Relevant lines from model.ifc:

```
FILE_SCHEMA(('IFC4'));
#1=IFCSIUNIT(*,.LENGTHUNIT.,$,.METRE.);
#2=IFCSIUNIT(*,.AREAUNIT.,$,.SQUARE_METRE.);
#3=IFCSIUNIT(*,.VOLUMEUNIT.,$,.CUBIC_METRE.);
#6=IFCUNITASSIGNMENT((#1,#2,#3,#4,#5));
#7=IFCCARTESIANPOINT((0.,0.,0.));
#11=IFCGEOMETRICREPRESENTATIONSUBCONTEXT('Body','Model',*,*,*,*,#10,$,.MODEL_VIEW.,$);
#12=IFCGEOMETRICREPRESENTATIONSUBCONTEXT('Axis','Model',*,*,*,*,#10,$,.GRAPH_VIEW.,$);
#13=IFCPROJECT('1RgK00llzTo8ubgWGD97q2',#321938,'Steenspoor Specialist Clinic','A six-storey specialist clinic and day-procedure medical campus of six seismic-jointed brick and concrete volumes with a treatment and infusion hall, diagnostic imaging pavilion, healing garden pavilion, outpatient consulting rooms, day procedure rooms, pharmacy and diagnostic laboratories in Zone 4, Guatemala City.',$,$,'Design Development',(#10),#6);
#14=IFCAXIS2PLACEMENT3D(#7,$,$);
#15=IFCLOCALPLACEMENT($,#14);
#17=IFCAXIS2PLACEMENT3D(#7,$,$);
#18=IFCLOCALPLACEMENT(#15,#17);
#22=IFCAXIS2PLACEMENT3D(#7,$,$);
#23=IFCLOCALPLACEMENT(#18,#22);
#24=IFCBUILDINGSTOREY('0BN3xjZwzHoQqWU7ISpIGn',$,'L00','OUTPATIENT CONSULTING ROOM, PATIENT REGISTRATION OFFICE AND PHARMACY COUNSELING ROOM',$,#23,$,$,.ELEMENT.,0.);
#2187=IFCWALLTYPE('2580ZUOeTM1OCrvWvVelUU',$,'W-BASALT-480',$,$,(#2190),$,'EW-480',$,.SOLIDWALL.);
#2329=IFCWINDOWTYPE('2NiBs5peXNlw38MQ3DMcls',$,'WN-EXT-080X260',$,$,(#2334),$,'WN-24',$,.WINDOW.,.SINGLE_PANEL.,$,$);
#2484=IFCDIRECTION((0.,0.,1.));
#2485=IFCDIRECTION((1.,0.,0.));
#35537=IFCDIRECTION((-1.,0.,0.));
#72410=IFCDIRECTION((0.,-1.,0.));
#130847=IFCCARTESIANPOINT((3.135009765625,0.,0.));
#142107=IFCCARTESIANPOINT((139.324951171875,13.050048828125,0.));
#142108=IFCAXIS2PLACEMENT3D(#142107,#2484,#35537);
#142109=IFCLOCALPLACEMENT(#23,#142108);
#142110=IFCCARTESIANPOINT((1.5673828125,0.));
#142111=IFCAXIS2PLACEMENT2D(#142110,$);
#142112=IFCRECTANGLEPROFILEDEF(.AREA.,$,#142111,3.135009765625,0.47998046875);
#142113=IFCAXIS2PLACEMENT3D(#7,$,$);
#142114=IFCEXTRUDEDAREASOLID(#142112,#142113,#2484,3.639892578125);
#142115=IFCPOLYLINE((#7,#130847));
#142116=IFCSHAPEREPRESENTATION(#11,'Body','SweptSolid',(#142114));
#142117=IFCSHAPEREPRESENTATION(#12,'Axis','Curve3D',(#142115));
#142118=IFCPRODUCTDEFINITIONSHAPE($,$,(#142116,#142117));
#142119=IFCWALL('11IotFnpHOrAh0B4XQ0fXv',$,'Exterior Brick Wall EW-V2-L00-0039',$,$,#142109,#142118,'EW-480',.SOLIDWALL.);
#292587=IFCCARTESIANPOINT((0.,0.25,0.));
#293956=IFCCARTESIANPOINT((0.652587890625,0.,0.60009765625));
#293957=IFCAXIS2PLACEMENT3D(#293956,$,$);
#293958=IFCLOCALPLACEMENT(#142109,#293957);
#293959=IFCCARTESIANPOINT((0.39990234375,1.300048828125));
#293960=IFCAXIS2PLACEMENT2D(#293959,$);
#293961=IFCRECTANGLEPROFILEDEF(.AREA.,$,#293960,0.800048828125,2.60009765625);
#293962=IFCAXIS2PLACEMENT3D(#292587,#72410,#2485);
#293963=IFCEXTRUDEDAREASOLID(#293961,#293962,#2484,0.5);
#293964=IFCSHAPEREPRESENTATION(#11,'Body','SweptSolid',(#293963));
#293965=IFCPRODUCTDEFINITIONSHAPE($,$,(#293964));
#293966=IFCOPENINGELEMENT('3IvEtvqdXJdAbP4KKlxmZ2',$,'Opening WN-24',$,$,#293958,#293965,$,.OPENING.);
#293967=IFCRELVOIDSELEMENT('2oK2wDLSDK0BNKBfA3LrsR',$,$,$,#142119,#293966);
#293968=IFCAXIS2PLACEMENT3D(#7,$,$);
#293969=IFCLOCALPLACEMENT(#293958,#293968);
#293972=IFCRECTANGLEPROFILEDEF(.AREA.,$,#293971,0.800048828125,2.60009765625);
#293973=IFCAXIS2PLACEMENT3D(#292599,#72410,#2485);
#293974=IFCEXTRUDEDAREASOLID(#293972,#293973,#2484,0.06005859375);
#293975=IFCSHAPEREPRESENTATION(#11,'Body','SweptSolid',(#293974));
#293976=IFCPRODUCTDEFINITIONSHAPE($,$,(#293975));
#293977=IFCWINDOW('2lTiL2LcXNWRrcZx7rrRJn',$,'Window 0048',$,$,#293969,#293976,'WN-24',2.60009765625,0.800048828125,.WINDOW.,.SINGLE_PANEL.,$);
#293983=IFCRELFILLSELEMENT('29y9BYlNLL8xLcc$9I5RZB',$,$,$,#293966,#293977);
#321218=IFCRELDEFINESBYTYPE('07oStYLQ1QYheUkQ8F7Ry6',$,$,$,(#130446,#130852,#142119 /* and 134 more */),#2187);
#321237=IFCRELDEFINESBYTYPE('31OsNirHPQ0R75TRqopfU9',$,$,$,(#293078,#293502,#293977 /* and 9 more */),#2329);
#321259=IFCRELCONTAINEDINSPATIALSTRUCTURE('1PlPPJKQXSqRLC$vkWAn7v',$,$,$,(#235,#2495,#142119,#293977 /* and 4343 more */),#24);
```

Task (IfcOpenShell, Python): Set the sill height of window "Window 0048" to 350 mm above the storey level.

```python
import numpy as np
import ifcopenshell
import ifcopenshell.api.geometry
import ifcopenshell.geom
import ifcopenshell.util.element
import ifcopenshell.util.placement
import ifcopenshell.util.shape
import ifcopenshell.util.unit

model = ifcopenshell.open("model.ifc")
unit_scale = ifcopenshell.util.unit.calculate_unit_scale(model)

window = model.by_guid("2lTiL2LcXNWRrcZx7rrRJn")
opening = window.FillsVoids[0].RelatingOpeningElement
storey = ifcopenshell.util.element.get_container(window, ifc_class="IfcBuildingStorey")
level = ifcopenshell.util.placement.get_local_placement(storey.ObjectPlacement)[2, 3]

# The opening's origin need not be at the sill, so measure its lowest point.
shape = ifcopenshell.geom.create_shape(ifcopenshell.geom.settings(), opening)
bottom = ifcopenshell.util.shape.get_shape_bottom_elevation(shape, shape.geometry) / unit_scale
dz = level + 0.35 - bottom

shift = np.array([0.0, 0.0, dz])
# The window is placed relative to its opening, so it follows when the opening moves.
matrix = ifcopenshell.util.placement.get_local_placement(opening.ObjectPlacement)
matrix[:3, 3] += shift
ifcopenshell.api.geometry.edit_object_placement(
    model, product=opening, matrix=matrix, is_si=False, should_transform_children=True
)

print(f"moved by {dz * unit_scale:+.3f} m")

model.write("model_rev.ifc")
```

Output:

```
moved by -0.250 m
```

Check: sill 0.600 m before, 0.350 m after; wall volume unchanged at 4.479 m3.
